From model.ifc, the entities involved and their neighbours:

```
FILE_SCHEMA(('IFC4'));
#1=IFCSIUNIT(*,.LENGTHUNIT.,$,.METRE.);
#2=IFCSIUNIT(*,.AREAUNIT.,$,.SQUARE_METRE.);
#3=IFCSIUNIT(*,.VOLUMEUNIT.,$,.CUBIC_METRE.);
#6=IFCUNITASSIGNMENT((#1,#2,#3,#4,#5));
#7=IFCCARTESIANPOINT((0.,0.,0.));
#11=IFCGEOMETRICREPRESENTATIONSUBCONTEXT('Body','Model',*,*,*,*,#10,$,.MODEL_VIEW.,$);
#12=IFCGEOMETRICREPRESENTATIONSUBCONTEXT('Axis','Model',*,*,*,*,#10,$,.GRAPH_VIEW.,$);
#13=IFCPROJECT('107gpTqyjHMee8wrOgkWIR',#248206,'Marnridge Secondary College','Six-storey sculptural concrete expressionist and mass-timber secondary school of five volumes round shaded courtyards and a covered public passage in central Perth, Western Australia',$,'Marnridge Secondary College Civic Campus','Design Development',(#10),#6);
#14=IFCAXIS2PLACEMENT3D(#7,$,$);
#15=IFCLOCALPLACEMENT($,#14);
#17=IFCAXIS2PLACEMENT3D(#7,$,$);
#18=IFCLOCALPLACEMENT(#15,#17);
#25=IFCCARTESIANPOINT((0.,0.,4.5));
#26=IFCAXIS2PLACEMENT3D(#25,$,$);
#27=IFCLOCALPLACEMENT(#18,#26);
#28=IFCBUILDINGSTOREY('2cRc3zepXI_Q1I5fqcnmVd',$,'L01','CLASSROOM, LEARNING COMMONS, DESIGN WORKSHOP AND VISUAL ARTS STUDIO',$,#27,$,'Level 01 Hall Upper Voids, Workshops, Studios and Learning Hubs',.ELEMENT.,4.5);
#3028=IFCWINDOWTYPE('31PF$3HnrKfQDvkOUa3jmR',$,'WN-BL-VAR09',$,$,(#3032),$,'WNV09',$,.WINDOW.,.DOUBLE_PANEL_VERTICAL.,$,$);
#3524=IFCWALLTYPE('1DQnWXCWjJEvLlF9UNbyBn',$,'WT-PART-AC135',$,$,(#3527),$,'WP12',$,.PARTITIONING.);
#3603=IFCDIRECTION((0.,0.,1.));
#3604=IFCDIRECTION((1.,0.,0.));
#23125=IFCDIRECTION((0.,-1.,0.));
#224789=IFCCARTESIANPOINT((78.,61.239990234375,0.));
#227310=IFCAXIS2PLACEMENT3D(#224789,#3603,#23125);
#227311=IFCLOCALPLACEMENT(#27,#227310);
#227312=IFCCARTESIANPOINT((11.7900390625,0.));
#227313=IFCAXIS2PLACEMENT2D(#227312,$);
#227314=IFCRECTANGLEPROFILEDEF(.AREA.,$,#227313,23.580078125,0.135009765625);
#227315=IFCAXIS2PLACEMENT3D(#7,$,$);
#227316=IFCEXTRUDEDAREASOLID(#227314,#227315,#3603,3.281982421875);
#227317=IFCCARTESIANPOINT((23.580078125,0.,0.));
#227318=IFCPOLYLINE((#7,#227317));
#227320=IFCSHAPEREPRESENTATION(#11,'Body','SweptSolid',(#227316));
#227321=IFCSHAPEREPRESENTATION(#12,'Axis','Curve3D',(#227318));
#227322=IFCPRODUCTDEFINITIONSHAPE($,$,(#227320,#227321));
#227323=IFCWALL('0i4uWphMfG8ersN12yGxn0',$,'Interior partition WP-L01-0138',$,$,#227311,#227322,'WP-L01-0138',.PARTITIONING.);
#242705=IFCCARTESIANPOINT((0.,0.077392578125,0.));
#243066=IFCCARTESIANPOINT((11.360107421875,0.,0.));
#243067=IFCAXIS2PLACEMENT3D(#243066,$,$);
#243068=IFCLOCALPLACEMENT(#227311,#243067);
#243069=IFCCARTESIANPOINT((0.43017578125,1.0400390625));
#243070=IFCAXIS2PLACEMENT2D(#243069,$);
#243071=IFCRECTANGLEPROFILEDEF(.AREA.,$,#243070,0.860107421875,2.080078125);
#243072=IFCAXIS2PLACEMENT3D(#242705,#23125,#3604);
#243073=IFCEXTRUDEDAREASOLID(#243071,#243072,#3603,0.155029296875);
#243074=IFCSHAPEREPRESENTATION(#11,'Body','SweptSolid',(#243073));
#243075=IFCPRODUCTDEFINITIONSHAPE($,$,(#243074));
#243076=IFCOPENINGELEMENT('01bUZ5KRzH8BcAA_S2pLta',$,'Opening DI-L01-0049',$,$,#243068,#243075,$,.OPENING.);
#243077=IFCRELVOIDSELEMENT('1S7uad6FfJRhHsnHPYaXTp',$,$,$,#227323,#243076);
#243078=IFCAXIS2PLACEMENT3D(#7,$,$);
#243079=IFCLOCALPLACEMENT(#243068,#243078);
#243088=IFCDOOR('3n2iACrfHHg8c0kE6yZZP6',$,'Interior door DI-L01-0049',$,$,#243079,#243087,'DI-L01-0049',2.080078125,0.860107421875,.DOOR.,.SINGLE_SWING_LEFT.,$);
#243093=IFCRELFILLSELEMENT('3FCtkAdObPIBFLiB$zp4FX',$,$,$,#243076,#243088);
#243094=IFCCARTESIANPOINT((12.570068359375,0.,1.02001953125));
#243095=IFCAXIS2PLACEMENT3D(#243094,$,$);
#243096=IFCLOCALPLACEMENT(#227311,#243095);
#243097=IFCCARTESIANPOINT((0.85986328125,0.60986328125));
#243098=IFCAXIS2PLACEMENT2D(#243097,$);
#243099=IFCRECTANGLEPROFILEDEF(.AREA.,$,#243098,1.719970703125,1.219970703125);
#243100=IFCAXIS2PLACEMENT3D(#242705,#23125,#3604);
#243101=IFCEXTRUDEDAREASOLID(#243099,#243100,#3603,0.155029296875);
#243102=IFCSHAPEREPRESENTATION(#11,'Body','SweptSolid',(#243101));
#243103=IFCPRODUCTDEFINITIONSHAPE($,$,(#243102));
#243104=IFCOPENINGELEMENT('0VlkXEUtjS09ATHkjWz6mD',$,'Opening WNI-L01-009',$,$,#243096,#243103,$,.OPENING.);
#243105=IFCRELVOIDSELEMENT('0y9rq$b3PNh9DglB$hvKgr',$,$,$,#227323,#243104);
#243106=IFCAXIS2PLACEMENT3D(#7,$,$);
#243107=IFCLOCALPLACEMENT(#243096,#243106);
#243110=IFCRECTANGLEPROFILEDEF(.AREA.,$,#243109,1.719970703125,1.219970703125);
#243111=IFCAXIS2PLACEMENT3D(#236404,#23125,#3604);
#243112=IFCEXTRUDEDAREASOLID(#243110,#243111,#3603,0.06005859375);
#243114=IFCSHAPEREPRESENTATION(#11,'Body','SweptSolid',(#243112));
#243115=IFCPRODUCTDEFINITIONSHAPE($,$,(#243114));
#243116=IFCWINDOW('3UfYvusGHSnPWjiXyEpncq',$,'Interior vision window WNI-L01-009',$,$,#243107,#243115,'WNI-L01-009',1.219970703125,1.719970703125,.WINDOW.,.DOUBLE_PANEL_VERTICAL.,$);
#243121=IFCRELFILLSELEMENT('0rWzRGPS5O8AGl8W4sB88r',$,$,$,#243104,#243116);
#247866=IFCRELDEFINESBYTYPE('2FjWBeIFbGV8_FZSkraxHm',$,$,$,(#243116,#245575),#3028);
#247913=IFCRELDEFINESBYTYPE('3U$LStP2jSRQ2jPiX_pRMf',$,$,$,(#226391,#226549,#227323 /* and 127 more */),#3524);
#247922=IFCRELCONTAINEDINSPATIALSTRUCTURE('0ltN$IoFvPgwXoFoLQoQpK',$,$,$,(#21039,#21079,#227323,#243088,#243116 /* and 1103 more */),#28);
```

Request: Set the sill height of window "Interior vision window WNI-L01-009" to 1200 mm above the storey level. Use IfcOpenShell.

```python
import numpy as np
import ifcopenshell
import ifcopenshell.api.geometry
import ifcopenshell.geom
import ifcopenshell.util.element
import ifcopenshell.util.placement
import ifcopenshell.util.shape
import ifcopenshell.util.unit

model = ifcopenshell.open("model.ifc")
unit_scale = ifcopenshell.util.unit.calculate_unit_scale(model)

window = model.by_guid("3UfYvusGHSnPWjiXyEpncq")
opening = window.FillsVoids[0].RelatingOpeningElement
storey = ifcopenshell.util.element.get_container(window, ifc_class="IfcBuildingStorey")
level = ifcopenshell.util.placement.get_local_placement(storey.ObjectPlacement)[2, 3]

# The opening's origin need not be at the sill, so measure its lowest point.
shape = ifcopenshell.geom.create_shape(ifcopenshell.geom.settings(), opening)
bottom = ifcopenshell.util.shape.get_shape_bottom_elevation(shape, shape.geometry) / unit_scale
dz = level + 1.2 / unit_scale - bottom

shift = np.array([0.0, 0.0, dz])
# The window is placed relative to its opening, so it follows when the opening moves.
matrix = ifcopenshell.util.placement.get_local_placement(opening.ObjectPlacement)
matrix[:3, 3] += shift
ifcopenshell.api.geometry.edit_object_placement(
    model, product=opening, matrix=matrix, is_si=False, should_transform_children=True
)

print(f"moved by {dz * unit_scale:+.3f} m")

model.write("model_v2.ifc")
```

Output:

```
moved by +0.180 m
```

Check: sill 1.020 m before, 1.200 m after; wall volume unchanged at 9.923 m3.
